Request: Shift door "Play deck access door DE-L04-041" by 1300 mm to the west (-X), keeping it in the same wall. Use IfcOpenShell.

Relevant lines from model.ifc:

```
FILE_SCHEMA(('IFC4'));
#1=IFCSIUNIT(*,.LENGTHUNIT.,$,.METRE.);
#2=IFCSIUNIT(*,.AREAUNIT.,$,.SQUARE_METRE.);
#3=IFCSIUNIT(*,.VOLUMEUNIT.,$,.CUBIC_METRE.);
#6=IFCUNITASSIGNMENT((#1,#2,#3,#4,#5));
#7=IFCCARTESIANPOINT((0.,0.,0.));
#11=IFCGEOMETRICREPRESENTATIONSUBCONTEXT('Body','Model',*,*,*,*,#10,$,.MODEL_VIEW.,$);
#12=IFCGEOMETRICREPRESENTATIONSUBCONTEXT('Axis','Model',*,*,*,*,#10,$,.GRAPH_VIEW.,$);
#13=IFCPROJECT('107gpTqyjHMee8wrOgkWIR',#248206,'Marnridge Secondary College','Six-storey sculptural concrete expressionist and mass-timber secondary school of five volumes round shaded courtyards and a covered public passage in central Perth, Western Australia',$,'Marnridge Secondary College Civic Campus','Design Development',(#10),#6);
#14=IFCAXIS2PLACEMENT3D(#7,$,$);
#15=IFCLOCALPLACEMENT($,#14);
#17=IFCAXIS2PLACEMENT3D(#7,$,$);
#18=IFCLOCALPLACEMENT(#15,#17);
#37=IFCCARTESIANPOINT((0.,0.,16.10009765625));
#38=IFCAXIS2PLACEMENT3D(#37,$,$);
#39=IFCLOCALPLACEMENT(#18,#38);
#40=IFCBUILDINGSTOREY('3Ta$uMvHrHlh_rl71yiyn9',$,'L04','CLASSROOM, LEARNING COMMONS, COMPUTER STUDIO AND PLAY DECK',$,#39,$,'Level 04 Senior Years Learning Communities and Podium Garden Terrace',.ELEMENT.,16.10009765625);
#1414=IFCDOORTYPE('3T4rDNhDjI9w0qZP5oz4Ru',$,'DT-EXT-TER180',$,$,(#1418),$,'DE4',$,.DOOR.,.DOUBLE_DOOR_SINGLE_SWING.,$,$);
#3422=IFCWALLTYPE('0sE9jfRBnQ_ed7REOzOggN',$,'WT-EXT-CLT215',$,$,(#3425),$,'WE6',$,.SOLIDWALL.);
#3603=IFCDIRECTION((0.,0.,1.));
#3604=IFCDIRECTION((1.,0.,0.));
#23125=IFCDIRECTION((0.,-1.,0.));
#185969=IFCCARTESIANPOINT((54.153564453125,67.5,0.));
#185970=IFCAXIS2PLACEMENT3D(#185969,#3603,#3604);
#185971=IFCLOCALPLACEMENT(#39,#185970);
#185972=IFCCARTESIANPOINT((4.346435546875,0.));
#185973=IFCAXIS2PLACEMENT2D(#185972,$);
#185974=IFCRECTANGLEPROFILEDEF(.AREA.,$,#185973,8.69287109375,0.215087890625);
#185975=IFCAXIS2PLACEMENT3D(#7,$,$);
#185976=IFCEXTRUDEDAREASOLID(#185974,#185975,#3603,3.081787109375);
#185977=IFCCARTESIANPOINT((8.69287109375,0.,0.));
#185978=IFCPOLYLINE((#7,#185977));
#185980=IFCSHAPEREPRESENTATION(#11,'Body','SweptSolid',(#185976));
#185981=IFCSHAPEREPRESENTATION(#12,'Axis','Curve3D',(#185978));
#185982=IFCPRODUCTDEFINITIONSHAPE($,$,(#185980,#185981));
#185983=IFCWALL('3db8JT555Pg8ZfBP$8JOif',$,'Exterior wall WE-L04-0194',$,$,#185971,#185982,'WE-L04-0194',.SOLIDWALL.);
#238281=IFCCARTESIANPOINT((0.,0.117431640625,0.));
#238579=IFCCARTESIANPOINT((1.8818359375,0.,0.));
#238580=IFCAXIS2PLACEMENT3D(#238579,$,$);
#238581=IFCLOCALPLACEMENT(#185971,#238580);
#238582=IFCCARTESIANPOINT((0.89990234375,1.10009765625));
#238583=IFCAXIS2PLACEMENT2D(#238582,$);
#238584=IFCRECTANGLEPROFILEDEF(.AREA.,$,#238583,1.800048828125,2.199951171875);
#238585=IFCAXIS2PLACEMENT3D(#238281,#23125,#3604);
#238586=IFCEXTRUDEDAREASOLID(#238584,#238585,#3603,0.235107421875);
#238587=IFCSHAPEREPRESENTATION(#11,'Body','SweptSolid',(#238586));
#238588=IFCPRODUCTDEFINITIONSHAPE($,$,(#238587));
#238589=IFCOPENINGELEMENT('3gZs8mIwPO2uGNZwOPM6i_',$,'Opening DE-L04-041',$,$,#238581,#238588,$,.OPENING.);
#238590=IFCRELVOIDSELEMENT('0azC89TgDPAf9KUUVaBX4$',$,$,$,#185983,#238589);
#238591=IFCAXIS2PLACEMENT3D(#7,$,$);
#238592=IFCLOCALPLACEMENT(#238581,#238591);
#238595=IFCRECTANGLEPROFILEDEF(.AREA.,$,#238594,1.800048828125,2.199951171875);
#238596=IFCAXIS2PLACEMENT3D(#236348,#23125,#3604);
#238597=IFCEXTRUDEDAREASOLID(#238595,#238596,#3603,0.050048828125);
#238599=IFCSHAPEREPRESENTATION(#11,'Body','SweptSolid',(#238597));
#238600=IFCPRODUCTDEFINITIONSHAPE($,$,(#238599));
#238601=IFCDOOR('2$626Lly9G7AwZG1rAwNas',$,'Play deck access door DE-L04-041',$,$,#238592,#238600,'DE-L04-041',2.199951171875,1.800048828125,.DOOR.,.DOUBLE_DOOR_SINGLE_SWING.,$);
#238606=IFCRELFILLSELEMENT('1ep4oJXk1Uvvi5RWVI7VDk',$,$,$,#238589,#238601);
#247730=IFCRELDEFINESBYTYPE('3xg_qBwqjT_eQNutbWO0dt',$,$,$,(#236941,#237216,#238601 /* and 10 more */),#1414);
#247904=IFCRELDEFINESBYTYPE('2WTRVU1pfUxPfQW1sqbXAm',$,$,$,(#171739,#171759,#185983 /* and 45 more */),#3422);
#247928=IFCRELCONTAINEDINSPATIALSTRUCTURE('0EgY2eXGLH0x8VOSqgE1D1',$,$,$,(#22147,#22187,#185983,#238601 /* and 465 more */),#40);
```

```python
import ifcopenshell
import ifcopenshell.api.geometry
import ifcopenshell.util.placement

model = ifcopenshell.open("model.ifc")

door = model.by_guid("2$626Lly9G7AwZG1rAwNas")
opening = door.FillsVoids[0].RelatingOpeningElement
wall = opening.VoidsElements[0].RelatingBuildingElement

wall_matrix = ifcopenshell.util.placement.get_local_placement(wall.ObjectPlacement)
shift = wall_matrix[:3, 0] * -1.3
before = ifcopenshell.util.placement.get_local_placement(door.ObjectPlacement)[:3, 3].copy()

# The door is placed relative to its opening, so it follows when the opening moves.
matrix = ifcopenshell.util.placement.get_local_placement(opening.ObjectPlacement)
matrix[:3, 3] += shift
ifcopenshell.api.geometry.edit_object_placement(
    model, product=opening, matrix=matrix, is_si=False, should_transform_children=True
)

after = ifcopenshell.util.placement.get_local_placement(door.ObjectPlacement)[:3, 3]
print("door moved by", (after - before).round(3) + 0.0)

model.write("model-out.ifc")
```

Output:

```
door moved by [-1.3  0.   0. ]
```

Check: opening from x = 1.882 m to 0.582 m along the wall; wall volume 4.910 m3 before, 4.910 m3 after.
